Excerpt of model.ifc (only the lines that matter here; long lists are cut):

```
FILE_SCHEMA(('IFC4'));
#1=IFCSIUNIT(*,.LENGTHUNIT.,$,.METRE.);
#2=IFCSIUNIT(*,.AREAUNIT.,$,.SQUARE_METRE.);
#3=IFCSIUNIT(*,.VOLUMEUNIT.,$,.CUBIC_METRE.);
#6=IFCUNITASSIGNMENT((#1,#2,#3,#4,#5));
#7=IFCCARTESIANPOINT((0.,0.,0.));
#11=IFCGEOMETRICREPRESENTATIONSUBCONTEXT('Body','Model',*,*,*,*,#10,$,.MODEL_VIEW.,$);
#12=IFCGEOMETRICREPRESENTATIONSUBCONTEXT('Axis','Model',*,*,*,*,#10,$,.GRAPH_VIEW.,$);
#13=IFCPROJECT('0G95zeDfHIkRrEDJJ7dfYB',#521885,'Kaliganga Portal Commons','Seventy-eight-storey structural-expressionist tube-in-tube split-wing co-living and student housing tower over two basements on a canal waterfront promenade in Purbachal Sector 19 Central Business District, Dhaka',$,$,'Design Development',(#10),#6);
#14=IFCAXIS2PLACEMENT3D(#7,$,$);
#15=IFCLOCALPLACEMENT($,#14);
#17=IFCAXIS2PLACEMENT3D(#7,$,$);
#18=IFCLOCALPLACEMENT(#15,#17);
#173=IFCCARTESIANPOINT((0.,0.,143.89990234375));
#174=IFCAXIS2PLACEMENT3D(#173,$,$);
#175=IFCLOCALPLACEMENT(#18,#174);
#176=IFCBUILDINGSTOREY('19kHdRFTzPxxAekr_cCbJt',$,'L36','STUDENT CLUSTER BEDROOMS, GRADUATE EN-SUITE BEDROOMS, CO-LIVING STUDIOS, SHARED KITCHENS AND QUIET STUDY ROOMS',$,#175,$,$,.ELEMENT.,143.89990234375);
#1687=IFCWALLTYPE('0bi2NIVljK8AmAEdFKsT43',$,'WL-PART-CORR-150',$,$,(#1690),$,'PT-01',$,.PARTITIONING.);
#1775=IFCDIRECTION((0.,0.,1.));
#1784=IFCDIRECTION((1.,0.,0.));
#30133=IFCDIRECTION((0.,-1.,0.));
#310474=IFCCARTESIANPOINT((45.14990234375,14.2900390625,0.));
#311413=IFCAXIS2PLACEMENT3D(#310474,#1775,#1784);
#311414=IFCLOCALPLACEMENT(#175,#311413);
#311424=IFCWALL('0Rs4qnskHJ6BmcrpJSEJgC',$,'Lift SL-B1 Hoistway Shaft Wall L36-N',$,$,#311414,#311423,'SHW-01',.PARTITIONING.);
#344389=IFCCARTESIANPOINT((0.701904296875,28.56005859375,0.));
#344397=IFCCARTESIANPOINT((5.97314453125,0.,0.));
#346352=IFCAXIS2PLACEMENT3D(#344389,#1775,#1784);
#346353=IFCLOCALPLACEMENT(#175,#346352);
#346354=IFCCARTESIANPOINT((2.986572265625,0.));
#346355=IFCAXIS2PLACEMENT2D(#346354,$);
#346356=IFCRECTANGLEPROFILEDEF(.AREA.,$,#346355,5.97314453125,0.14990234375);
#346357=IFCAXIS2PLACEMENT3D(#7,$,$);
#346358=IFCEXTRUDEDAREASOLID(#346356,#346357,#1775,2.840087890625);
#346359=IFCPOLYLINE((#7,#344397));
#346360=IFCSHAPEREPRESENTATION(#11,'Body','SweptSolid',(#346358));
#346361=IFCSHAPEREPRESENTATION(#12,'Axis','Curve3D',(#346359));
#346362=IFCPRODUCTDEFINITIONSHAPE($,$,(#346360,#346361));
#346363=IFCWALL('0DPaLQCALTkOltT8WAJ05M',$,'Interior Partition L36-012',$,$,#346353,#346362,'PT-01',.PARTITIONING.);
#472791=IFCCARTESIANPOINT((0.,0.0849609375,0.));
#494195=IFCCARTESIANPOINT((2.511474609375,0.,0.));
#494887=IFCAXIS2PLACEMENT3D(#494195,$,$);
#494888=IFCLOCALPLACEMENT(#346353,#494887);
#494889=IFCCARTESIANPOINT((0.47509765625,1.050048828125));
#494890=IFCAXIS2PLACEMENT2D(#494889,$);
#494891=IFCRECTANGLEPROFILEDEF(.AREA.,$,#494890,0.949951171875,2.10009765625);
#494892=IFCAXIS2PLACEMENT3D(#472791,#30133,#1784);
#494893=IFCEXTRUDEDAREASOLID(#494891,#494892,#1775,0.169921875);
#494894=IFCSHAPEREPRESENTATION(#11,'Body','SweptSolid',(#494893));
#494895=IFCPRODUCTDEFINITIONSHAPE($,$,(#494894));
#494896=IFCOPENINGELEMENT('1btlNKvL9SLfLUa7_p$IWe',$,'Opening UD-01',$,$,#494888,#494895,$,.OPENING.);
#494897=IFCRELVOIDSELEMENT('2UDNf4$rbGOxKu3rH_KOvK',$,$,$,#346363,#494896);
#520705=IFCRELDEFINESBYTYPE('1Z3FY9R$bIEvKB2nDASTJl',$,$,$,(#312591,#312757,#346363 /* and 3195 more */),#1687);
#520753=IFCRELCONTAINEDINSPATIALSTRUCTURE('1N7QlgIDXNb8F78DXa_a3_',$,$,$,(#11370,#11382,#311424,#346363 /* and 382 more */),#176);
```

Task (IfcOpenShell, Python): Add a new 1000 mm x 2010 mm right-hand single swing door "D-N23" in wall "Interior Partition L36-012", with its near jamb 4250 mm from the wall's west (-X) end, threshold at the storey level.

```python
import numpy as np
import ifcopenshell
import ifcopenshell.api.feature
import ifcopenshell.api.geometry
import ifcopenshell.api.root
import ifcopenshell.api.spatial
import ifcopenshell.geom
import ifcopenshell.util.element
import ifcopenshell.util.placement
import ifcopenshell.util.representation
import ifcopenshell.util.shape
import ifcopenshell.util.unit

model = ifcopenshell.open("model.ifc")
unit_scale = ifcopenshell.util.unit.calculate_unit_scale(model)
settings = ifcopenshell.geom.settings()


def volume(element):
    """Net volume in cubic metres, openings subtracted."""
    shape = ifcopenshell.geom.create_shape(settings, element)
    return ifcopenshell.util.shape.get_volume(shape.geometry)


wall = model.by_guid("0DPaLQCALTkOltT8WAJ05M")
storey = ifcopenshell.util.element.get_container(wall, ifc_class="IfcBuildingStorey")
context = ifcopenshell.util.representation.get_context(model, "Model", "Body", "MODEL_VIEW")
before = volume(wall)

width, height, from_end, sill = 1, 2.01, 4.25, 0.0  # metres

# The wall runs along its own X axis, and the end named is its -X end.
wall_shape = ifcopenshell.geom.create_shape(settings, wall)
x, y, z = ifcopenshell.util.shape.get_vertices(wall_shape.geometry).T
start = x.min() + from_end
face, thickness = float(y.min()), float(y.max() - y.min())
wall_matrix = ifcopenshell.util.placement.get_local_placement(wall.ObjectPlacement)
level = ifcopenshell.util.placement.get_local_placement(storey.ObjectPlacement)[2, 3]


def in_wall(x, y):
    """Placement at x, y metres in the wall's axes, at sill height."""
    matrix = wall_matrix.copy()
    matrix[:, 3] = wall_matrix @ np.array([x / unit_scale, y / unit_scale, 0.0, 1.0])
    matrix[2, 3] = level + sill / unit_scale
    return matrix


# Opening: a box that overshoots both wall faces by 50 mm.
opening = ifcopenshell.api.root.create_entity(model, ifc_class="IfcOpeningElement", predefined_type="OPENING")
box = ifcopenshell.api.geometry.add_wall_representation(
    model, context=context, length=width, height=height, thickness=thickness + 0.1
)
ifcopenshell.api.geometry.assign_representation(model, product=opening, representation=box)
ifcopenshell.api.geometry.edit_object_placement(model, product=opening, matrix=in_wall(start, face - 0.05), is_si=False)
ifcopenshell.api.feature.add_feature(model, feature=opening, element=wall)

door = ifcopenshell.api.root.create_entity(model, ifc_class="IfcDoor", name="D-N23", predefined_type="DOOR")
door.OverallWidth, door.OverallHeight = width / unit_scale, height / unit_scale
door.OperationType = "SINGLE_SWING_RIGHT"
body = ifcopenshell.api.geometry.add_door_representation(
    model,
    context=context,
    overall_width=door.OverallWidth,
    overall_height=door.OverallHeight,
    operation_type="SINGLE_SWING_RIGHT",
    lining_properties={"LiningDepth": thickness / unit_scale, "ThresholdDepth": thickness / unit_scale},
)
ifcopenshell.api.geometry.assign_representation(model, product=door, representation=body)
ifcopenshell.api.spatial.assign_container(model, products=[door], relating_structure=storey)
ifcopenshell.api.feature.add_filling(model, opening=opening, element=door)

# The lining spans the wall, so the door starts at the wall face.
ifcopenshell.api.geometry.edit_object_placement(model, product=door, matrix=in_wall(start, face), is_si=False)

after = volume(wall)

print(f"wall volume {before:.3f} -> {after:.3f} m3")

model.write("model-out.ifc")
```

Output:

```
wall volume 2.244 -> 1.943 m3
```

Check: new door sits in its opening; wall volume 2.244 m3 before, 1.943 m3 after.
